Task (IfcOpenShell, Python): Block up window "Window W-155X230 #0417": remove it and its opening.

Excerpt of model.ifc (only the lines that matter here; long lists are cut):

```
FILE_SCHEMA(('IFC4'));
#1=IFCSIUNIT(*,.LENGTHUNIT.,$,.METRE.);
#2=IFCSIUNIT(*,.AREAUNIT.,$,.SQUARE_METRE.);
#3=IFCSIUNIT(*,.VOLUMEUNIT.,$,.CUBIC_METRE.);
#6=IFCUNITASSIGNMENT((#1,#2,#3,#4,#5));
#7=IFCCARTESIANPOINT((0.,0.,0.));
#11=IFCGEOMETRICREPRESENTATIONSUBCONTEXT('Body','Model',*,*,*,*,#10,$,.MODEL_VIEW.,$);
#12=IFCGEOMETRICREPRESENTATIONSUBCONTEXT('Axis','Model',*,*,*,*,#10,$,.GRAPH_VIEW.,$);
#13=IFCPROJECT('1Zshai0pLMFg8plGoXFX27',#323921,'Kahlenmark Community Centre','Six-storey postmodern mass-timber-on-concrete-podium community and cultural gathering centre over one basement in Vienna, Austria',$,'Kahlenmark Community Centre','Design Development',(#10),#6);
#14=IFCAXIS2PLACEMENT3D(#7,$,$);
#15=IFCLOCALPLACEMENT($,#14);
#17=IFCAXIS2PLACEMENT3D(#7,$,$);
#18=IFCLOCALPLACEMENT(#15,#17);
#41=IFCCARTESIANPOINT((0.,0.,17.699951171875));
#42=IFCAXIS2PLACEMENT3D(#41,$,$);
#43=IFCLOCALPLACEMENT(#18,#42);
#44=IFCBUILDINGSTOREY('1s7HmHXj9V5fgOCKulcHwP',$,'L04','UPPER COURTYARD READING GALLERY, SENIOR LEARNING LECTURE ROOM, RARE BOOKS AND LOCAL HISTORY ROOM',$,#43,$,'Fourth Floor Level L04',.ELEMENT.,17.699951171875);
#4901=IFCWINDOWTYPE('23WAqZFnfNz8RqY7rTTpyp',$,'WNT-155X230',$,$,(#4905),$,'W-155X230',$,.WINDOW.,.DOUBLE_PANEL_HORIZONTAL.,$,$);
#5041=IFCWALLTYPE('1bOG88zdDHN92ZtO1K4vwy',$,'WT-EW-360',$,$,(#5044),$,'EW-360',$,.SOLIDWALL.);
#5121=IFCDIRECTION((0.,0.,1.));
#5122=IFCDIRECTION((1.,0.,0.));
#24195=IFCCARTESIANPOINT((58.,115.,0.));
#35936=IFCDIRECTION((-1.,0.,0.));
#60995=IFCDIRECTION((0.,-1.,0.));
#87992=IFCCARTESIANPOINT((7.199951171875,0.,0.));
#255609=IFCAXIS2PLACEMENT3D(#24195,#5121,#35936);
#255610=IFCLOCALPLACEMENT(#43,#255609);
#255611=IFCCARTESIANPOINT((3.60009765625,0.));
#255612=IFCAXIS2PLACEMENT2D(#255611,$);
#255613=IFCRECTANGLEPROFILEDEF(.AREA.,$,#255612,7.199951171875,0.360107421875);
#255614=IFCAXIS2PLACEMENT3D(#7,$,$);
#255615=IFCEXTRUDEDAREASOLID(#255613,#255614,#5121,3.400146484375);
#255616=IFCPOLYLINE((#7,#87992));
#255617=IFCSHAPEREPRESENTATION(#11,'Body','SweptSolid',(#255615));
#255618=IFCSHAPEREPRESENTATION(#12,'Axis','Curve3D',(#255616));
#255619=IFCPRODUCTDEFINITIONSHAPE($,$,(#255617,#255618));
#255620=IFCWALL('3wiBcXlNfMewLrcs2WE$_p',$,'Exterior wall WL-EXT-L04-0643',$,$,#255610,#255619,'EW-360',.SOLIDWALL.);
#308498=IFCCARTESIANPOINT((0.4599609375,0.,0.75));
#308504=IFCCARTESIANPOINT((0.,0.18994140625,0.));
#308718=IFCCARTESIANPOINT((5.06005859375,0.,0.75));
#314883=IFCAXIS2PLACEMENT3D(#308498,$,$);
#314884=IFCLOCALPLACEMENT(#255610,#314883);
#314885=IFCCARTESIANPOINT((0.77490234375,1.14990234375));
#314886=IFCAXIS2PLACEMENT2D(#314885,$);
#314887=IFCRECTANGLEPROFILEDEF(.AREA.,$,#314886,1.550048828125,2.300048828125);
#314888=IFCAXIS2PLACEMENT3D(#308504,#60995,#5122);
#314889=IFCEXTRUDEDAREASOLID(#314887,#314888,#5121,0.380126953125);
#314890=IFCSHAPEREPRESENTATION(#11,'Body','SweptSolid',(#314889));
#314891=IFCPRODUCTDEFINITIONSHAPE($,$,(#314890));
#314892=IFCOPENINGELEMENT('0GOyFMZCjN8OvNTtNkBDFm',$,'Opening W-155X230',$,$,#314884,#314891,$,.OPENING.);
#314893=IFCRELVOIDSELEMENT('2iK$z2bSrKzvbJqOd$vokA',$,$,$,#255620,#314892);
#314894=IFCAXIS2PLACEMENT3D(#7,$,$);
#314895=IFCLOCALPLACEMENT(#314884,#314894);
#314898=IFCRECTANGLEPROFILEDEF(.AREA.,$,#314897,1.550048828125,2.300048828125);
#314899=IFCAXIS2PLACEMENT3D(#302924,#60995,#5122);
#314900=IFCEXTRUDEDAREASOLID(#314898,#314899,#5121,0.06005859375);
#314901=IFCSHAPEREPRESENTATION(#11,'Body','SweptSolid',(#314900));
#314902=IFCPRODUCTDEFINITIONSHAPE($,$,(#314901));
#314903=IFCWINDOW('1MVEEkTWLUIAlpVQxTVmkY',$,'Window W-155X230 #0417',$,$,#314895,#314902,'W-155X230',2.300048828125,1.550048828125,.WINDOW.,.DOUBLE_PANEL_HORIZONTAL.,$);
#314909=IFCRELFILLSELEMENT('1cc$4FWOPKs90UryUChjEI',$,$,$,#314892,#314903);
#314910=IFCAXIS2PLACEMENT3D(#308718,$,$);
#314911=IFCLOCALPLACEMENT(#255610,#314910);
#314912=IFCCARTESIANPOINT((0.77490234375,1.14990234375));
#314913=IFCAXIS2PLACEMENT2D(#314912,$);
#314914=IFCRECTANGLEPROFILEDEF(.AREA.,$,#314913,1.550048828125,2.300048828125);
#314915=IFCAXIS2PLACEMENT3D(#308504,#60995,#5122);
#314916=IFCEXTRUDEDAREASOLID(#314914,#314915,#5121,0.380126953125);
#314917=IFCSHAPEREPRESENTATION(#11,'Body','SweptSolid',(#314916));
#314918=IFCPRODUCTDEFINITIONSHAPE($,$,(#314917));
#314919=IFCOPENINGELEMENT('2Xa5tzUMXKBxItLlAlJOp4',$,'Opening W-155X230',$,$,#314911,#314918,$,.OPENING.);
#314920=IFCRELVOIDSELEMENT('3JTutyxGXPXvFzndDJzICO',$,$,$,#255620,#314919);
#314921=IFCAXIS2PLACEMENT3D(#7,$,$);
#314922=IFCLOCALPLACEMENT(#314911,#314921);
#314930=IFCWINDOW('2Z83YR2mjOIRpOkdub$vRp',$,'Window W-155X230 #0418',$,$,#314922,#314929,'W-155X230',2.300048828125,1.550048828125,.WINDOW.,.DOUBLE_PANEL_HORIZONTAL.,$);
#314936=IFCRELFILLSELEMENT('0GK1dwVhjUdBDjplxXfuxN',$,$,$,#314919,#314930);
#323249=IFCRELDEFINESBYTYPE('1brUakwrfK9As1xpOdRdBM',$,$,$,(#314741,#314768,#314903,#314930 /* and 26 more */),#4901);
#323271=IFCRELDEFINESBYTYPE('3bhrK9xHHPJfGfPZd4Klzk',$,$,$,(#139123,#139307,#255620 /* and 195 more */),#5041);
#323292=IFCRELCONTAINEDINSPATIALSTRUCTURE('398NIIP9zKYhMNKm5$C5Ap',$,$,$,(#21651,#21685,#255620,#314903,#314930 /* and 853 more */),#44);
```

```python
import ifcopenshell
import ifcopenshell.api.feature
import ifcopenshell.api.root
import ifcopenshell.geom
import ifcopenshell.util.shape

model = ifcopenshell.open("model.ifc")
settings = ifcopenshell.geom.settings()


def volume(element):
    """Net volume in cubic metres, openings subtracted."""
    shape = ifcopenshell.geom.create_shape(settings, element)
    return ifcopenshell.util.shape.get_volume(shape.geometry)


window = model.by_guid("1MVEEkTWLUIAlpVQxTVmkY")
opening = window.FillsVoids[0].RelatingOpeningElement
wall = opening.VoidsElements[0].RelatingBuildingElement
before = volume(wall)

ifcopenshell.api.root.remove_product(model, product=window)
ifcopenshell.api.feature.remove_feature(model, feature=opening)

after = volume(wall)

print(f"wall volume {before:.3f} -> {after:.3f} m3")

model.write("model_edited.ifc")
```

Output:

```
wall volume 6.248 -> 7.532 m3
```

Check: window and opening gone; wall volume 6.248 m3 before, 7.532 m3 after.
